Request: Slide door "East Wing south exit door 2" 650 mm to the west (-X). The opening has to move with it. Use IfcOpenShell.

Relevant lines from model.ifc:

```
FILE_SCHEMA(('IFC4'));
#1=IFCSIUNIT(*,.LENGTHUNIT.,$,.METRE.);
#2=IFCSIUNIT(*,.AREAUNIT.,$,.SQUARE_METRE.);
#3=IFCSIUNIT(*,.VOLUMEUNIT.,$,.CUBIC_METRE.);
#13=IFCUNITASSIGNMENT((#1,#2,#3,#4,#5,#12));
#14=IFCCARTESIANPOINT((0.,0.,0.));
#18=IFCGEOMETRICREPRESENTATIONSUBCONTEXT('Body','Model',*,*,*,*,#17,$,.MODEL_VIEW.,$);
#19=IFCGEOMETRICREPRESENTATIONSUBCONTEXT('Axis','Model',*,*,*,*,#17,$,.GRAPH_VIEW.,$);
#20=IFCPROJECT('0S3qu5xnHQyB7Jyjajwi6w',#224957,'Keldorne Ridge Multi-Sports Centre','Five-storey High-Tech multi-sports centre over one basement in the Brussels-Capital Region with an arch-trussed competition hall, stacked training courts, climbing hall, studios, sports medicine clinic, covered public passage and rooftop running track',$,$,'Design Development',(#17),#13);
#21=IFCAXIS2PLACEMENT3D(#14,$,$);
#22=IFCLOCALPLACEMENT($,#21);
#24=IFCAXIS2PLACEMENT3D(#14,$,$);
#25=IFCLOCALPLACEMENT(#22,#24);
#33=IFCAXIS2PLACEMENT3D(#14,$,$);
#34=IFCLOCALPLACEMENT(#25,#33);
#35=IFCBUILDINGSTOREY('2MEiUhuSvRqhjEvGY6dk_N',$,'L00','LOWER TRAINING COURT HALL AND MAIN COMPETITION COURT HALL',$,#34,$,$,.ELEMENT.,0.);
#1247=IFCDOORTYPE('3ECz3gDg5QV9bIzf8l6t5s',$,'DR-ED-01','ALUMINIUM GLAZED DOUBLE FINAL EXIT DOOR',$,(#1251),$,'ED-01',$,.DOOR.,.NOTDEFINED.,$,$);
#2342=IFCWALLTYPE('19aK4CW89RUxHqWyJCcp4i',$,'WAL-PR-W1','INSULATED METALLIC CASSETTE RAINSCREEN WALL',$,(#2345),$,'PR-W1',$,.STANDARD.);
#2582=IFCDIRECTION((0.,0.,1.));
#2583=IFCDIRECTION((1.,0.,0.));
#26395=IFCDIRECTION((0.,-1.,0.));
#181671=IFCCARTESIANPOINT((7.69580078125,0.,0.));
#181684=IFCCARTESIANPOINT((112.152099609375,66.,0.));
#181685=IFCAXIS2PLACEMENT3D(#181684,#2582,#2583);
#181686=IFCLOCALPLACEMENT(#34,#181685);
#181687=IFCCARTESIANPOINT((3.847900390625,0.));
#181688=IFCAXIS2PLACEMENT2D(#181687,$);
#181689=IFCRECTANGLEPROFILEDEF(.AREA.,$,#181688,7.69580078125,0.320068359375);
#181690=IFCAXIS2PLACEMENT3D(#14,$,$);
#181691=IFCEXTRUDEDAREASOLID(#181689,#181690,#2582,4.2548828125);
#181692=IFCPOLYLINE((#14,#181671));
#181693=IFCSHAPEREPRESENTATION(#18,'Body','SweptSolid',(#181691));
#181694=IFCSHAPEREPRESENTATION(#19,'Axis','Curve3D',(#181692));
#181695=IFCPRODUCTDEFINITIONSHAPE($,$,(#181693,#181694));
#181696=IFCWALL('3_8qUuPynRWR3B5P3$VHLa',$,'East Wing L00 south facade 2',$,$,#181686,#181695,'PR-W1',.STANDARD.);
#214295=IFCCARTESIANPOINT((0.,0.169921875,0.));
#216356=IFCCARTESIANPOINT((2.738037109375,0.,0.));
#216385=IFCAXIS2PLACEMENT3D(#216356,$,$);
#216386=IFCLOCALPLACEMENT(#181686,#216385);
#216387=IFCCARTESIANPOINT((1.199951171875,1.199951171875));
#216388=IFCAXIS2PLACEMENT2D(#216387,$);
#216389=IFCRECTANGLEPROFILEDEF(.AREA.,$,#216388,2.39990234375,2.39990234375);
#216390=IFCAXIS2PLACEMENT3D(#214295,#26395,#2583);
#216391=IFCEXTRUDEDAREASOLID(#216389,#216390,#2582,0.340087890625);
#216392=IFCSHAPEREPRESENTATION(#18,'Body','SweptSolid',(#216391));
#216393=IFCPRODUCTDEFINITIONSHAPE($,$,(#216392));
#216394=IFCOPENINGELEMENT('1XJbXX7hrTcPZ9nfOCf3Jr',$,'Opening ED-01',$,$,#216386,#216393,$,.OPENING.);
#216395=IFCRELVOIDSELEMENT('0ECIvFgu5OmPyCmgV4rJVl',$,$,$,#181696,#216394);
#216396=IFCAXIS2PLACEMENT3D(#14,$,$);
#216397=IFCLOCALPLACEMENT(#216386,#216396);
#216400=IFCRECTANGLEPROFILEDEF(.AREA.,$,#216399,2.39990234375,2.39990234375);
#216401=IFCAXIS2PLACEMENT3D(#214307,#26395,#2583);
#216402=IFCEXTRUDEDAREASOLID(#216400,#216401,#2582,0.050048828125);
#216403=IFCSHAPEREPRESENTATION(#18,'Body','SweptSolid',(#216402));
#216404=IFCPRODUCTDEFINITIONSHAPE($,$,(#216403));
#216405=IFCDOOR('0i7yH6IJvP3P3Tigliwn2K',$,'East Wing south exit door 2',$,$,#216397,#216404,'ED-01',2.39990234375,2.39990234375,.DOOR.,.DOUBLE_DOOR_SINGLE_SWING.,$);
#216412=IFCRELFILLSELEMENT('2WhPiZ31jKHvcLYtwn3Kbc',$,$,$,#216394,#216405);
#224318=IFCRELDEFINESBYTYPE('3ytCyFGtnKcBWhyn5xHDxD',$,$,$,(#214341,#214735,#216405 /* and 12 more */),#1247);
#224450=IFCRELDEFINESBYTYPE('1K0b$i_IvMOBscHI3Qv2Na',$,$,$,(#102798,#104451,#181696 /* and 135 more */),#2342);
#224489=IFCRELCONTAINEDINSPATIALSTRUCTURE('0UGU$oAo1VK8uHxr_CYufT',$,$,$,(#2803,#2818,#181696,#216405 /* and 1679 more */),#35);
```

```python
import ifcopenshell
import ifcopenshell.api.geometry
import ifcopenshell.util.placement
import ifcopenshell.util.unit

model = ifcopenshell.open("model.ifc")
unit_scale = ifcopenshell.util.unit.calculate_unit_scale(model)

door = model.by_guid("0i7yH6IJvP3P3Tigliwn2K")
opening = door.FillsVoids[0].RelatingOpeningElement
wall = opening.VoidsElements[0].RelatingBuildingElement

wall_matrix = ifcopenshell.util.placement.get_local_placement(wall.ObjectPlacement)
shift = wall_matrix[:3, 0] * -0.65 / unit_scale
before = ifcopenshell.util.placement.get_local_placement(door.ObjectPlacement)[:3, 3].copy()

# The door is placed relative to its opening, so it follows when the opening moves.
matrix = ifcopenshell.util.placement.get_local_placement(opening.ObjectPlacement)
matrix[:3, 3] += shift
ifcopenshell.api.geometry.edit_object_placement(
    model, product=opening, matrix=matrix, is_si=False, should_transform_children=True
)

after = ifcopenshell.util.placement.get_local_placement(door.ObjectPlacement)[:3, 3]
print("door moved by", (after - before).round(3) + 0.0)

model.write("model-out.ifc")
```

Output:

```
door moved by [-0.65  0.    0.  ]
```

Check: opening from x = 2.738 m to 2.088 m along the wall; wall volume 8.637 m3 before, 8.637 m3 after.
